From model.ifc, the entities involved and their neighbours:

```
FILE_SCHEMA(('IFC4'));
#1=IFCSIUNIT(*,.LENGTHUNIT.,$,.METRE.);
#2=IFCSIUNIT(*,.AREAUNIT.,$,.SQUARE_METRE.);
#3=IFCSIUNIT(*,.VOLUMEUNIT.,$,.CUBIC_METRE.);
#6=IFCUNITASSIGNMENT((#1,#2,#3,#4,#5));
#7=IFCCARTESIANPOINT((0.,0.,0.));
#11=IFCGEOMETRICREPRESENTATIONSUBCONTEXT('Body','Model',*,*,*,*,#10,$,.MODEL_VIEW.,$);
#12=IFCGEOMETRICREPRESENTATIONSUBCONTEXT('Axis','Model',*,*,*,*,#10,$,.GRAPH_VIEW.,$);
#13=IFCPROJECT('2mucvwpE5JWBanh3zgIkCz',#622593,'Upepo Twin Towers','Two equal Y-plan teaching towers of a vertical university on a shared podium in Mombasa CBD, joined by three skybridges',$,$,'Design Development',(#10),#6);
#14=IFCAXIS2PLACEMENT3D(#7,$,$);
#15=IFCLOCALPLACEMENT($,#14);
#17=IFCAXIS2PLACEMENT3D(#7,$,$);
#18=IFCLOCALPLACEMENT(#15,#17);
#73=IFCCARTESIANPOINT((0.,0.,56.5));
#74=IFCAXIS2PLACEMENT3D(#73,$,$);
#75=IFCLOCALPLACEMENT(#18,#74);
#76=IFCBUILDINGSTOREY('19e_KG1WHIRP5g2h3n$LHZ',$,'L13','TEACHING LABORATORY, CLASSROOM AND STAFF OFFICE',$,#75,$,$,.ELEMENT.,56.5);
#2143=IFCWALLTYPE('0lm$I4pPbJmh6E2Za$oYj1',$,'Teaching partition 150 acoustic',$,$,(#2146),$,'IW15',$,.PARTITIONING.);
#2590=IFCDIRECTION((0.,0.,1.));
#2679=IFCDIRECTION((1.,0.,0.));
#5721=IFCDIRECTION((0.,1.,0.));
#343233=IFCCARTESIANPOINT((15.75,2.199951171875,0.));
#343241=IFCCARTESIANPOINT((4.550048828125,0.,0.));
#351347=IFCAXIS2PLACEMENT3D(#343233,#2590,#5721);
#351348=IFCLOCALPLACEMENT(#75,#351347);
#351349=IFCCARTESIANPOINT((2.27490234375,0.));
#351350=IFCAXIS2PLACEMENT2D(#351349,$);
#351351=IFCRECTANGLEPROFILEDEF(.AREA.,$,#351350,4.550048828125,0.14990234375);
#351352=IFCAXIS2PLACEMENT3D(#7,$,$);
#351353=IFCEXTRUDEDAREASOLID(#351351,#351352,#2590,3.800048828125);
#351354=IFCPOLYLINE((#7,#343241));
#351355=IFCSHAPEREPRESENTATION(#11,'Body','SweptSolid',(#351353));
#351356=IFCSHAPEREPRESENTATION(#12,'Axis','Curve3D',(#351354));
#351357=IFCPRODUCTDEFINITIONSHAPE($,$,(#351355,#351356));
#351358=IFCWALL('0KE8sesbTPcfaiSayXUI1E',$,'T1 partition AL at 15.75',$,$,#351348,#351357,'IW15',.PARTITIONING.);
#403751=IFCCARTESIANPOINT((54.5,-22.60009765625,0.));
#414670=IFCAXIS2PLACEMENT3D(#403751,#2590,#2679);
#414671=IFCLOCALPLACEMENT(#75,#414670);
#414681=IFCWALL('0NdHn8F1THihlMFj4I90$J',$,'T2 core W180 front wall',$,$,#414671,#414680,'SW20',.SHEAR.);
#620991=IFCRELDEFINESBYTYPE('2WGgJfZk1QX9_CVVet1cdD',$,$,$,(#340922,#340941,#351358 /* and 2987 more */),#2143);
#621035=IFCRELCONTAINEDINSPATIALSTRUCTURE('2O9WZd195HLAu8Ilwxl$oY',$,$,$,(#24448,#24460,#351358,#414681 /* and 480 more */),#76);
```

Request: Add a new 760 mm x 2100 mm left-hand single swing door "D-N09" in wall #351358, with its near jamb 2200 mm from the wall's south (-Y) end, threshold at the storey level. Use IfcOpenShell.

```python
import numpy as np
import ifcopenshell
import ifcopenshell.api.feature
import ifcopenshell.api.geometry
import ifcopenshell.api.root
import ifcopenshell.api.spatial
import ifcopenshell.geom
import ifcopenshell.util.element
import ifcopenshell.util.placement
import ifcopenshell.util.representation
import ifcopenshell.util.shape
import ifcopenshell.util.unit

model = ifcopenshell.open("model.ifc")
unit_scale = ifcopenshell.util.unit.calculate_unit_scale(model)
settings = ifcopenshell.geom.settings()


def volume(element):
    """Net volume in cubic metres, openings subtracted."""
    shape = ifcopenshell.geom.create_shape(settings, element)
    return ifcopenshell.util.shape.get_volume(shape.geometry)


wall = model.by_guid("0KE8sesbTPcfaiSayXUI1E")
storey = ifcopenshell.util.element.get_container(wall, ifc_class="IfcBuildingStorey")
context = ifcopenshell.util.representation.get_context(model, "Model", "Body", "MODEL_VIEW")
before = volume(wall)

width, height, from_end, sill = 0.76, 2.1, 2.2, 0.0  # metres

# The wall runs along its own X axis, and the end named is its -X end.
wall_shape = ifcopenshell.geom.create_shape(settings, wall)
x, y, z = ifcopenshell.util.shape.get_vertices(wall_shape.geometry).T
start = x.min() + from_end
face, thickness = float(y.min()), float(y.max() - y.min())
wall_matrix = ifcopenshell.util.placement.get_local_placement(wall.ObjectPlacement)
level = ifcopenshell.util.placement.get_local_placement(storey.ObjectPlacement)[2, 3]


def in_wall(x, y):
    """Placement at x, y metres in the wall's axes, at sill height."""
    matrix = wall_matrix.copy()
    matrix[:, 3] = wall_matrix @ np.array([x / unit_scale, y / unit_scale, 0.0, 1.0])
    matrix[2, 3] = level + sill / unit_scale
    return matrix


# Opening: a box that overshoots both wall faces by 50 mm.
opening = ifcopenshell.api.root.create_entity(model, ifc_class="IfcOpeningElement", predefined_type="OPENING")
box = ifcopenshell.api.geometry.add_wall_representation(
    model, context=context, length=width, height=height, thickness=thickness + 0.1
)
ifcopenshell.api.geometry.assign_representation(model, product=opening, representation=box)
ifcopenshell.api.geometry.edit_object_placement(model, product=opening, matrix=in_wall(start, face - 0.05), is_si=False)
ifcopenshell.api.feature.add_feature(model, feature=opening, element=wall)

door = ifcopenshell.api.root.create_entity(model, ifc_class="IfcDoor", name="D-N09", predefined_type="DOOR")
door.OverallWidth, door.OverallHeight = width / unit_scale, height / unit_scale
door.OperationType = "SINGLE_SWING_LEFT"
body = ifcopenshell.api.geometry.add_door_representation(
    model,
    context=context,
    overall_width=door.OverallWidth,
    overall_height=door.OverallHeight,
    operation_type="SINGLE_SWING_LEFT",
    lining_properties={"LiningDepth": thickness / unit_scale, "ThresholdDepth": thickness / unit_scale},
)
ifcopenshell.api.geometry.assign_representation(model, product=door, representation=body)
ifcopenshell.api.spatial.assign_container(model, products=[door], relating_structure=storey)
ifcopenshell.api.feature.add_filling(model, opening=opening, element=door)

# The lining spans the wall, so the door starts at the wall face.
ifcopenshell.api.geometry.edit_object_placement(model, product=door, matrix=in_wall(start, face), is_si=False)

after = volume(wall)

print(f"wall volume {before:.3f} -> {after:.3f} m3")

model.write("model_v2.ifc")
```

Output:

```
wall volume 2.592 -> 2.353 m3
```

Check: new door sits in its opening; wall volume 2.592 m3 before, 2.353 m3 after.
